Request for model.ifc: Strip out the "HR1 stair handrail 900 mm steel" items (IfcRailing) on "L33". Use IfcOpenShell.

First a look at what the model holds.

```python
import ifcopenshell
import ifcopenshell.util.element

model = ifcopenshell.open("model.ifc")
print(model.schema)
storey = next(s for s in model.by_type("IfcBuildingStorey") if s.Name == "L33")
railings = [e for e in ifcopenshell.util.element.get_decomposition(storey) if e.is_a("IfcRailing")]
seen = {}
for e in railings:
    element_type = ifcopenshell.util.element.get_type(e)
    name = element_type.Name if element_type not in (None, e) else None
    seen[name] = seen.get(name, 0) + 1
for name, count in sorted(seen.items(), key=str):
    print(count, "x", name)
```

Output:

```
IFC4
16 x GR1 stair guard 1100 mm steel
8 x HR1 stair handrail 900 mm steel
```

```python
import ifcopenshell
import ifcopenshell.api.root
import ifcopenshell.util.element

model = ifcopenshell.open("model.ifc")

storey = next(s for s in model.by_type("IfcBuildingStorey") if s.Name == "L33")
railings = [e for e in ifcopenshell.util.element.get_decomposition(storey) if e.is_a("IfcRailing")]
targets = [e for e in railings if (t := ifcopenshell.util.element.get_type(e)) not in (None, e) and t.Name == "HR1 stair handrail 900 mm steel"]

for e in targets:
    ifcopenshell.api.root.remove_product(model, product=e)
print(len(targets), "removed")

model.write("model_v2.ifc")
```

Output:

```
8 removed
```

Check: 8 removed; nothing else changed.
